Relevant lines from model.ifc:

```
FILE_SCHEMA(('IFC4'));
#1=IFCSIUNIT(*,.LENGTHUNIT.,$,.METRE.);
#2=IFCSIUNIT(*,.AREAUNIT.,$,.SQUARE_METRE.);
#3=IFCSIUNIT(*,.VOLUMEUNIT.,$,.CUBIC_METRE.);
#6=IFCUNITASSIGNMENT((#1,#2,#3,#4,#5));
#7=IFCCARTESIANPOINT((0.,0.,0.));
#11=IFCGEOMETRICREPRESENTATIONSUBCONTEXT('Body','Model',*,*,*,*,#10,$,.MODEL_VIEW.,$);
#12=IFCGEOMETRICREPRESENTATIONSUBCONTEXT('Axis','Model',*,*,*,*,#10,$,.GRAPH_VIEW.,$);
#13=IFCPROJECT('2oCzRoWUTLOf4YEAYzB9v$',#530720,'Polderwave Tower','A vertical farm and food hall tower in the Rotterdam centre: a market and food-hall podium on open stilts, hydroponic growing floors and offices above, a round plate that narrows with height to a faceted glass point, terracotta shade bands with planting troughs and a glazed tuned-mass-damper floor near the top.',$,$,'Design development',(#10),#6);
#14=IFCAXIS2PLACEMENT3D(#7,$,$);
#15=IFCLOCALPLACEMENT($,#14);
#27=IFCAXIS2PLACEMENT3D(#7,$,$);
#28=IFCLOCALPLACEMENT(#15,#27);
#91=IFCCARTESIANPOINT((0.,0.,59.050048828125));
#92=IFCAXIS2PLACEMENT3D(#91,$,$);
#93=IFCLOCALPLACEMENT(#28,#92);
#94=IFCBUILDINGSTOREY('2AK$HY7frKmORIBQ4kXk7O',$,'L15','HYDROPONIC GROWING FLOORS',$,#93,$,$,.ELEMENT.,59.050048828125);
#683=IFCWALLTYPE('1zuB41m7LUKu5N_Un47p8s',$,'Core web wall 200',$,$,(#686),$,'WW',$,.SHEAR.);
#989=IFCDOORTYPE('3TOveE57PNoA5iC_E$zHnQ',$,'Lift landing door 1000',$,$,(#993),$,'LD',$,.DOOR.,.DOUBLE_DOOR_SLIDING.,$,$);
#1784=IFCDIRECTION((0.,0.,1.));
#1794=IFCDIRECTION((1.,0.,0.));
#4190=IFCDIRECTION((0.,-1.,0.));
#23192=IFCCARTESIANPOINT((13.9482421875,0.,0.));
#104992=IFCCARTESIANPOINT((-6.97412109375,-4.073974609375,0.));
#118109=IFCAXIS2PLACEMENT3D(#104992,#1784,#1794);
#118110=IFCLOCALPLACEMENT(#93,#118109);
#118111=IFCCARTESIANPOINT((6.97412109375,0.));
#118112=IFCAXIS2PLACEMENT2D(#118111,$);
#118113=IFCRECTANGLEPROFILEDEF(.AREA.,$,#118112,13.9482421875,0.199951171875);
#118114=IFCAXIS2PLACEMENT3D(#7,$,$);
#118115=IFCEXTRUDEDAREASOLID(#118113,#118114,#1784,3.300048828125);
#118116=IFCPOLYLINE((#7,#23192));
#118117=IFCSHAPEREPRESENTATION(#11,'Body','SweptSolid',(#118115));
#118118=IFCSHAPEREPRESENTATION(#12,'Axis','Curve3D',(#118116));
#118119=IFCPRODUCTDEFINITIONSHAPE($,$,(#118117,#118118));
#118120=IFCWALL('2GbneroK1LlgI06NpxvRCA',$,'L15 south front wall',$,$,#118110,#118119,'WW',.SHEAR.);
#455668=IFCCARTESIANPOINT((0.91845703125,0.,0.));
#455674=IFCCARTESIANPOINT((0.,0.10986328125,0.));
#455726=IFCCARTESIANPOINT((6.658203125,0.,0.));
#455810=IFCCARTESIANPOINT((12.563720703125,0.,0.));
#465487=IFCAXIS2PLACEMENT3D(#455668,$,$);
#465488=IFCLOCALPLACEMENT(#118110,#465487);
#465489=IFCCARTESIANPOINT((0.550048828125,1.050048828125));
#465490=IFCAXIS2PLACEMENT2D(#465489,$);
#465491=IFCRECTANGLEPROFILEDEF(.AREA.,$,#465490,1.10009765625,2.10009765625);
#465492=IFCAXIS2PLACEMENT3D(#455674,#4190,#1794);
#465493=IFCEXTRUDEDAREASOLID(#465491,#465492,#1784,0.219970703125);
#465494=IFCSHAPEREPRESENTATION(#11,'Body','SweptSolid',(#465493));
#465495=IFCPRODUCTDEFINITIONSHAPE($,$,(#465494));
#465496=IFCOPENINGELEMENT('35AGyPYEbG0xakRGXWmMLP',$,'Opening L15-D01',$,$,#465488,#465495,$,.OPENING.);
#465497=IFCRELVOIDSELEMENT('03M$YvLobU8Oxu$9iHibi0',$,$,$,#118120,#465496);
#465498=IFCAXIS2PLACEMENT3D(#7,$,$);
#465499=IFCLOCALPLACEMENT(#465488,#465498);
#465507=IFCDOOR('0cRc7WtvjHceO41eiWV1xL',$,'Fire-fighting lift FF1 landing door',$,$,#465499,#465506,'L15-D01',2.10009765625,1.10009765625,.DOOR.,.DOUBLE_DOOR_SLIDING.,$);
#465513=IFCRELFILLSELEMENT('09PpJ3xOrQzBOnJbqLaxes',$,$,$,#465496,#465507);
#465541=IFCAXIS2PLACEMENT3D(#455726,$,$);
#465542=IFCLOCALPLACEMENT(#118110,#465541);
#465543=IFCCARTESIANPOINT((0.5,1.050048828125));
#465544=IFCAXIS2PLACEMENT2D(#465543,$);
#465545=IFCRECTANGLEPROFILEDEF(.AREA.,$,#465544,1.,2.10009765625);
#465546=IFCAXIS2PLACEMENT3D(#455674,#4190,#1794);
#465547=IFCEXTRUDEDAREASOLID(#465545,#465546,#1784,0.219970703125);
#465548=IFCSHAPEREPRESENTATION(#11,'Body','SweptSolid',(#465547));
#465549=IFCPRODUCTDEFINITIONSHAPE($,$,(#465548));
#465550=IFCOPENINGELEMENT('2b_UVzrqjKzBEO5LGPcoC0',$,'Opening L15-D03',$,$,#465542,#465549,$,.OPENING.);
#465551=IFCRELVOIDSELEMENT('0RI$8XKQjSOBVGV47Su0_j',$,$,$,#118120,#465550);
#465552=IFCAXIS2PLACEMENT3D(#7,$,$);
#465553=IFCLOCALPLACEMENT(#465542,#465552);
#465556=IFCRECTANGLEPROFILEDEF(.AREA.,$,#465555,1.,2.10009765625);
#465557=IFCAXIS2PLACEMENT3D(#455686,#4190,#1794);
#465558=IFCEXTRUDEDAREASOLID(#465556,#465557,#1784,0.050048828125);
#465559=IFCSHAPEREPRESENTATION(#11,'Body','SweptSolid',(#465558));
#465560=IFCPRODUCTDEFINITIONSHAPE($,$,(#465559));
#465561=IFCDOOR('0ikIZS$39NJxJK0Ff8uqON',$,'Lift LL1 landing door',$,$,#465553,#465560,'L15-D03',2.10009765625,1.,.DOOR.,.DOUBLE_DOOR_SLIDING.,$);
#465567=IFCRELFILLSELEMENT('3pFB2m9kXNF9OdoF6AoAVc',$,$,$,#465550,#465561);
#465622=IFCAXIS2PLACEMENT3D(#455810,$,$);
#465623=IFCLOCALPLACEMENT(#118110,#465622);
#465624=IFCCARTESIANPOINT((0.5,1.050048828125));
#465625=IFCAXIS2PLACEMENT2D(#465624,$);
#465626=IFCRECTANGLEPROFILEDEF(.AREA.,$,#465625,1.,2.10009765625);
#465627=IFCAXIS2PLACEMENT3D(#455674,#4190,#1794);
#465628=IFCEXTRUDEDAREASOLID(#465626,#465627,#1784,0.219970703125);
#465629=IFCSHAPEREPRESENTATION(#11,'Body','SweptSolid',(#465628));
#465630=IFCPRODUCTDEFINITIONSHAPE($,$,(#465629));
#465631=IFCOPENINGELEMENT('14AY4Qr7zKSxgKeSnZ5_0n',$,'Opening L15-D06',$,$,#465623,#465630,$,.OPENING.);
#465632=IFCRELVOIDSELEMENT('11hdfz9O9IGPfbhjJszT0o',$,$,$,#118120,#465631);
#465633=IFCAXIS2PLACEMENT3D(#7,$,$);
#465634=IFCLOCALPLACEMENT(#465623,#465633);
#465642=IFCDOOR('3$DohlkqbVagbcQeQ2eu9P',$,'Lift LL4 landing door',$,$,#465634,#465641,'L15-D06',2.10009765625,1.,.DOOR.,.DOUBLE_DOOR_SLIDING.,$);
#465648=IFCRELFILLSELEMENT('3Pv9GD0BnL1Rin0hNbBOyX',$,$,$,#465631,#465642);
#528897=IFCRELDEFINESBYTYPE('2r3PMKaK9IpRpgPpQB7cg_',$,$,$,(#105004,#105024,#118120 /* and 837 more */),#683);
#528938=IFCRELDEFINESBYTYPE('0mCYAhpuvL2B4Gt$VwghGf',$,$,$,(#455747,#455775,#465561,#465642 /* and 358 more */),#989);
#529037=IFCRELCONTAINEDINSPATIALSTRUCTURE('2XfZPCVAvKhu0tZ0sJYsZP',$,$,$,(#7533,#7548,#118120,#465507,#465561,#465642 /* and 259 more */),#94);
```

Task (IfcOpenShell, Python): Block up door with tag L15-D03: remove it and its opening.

```python
import ifcopenshell
import ifcopenshell.api.feature
import ifcopenshell.api.root
import ifcopenshell.geom
import ifcopenshell.util.shape

model = ifcopenshell.open("model.ifc")
settings = ifcopenshell.geom.settings()


def volume(element):
    """Net volume in cubic metres, openings subtracted."""
    shape = ifcopenshell.geom.create_shape(settings, element)
    return ifcopenshell.util.shape.get_volume(shape.geometry)


door = model.by_guid("0ikIZS$39NJxJK0Ff8uqON")
opening = door.FillsVoids[0].RelatingOpeningElement
wall = opening.VoidsElements[0].RelatingBuildingElement
before = volume(wall)

ifcopenshell.api.root.remove_product(model, product=door)
ifcopenshell.api.feature.remove_feature(model, feature=opening)

after = volume(wall)

print(f"wall volume {before:.3f} -> {after:.3f} m3")

model.write("model_edited.ifc")
```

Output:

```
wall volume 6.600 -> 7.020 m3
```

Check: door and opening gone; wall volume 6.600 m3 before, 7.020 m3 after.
